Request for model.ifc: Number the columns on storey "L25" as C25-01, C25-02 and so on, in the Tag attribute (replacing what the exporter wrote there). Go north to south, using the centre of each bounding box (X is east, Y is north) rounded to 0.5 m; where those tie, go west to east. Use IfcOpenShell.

First a look at what the model holds.

```python
import ifcopenshell
import ifcopenshell.util.element
import ifcopenshell.util.placement

model = ifcopenshell.open("model.ifc")
print(model.schema)
storey = next(s for s in model.by_type("IfcBuildingStorey") if s.Name == "L25")
columns = [e for e in ifcopenshell.util.element.get_decomposition(storey) if e.is_a("IfcColumn")]
for e in sorted(columns, key=lambda e: e.id()):
    origin = ifcopenshell.util.placement.get_local_placement(e.ObjectPlacement)[:3, 3]
    print(e.id(), e.Tag, e.Name, origin.round(2) + 0.0, sep=" | ")
```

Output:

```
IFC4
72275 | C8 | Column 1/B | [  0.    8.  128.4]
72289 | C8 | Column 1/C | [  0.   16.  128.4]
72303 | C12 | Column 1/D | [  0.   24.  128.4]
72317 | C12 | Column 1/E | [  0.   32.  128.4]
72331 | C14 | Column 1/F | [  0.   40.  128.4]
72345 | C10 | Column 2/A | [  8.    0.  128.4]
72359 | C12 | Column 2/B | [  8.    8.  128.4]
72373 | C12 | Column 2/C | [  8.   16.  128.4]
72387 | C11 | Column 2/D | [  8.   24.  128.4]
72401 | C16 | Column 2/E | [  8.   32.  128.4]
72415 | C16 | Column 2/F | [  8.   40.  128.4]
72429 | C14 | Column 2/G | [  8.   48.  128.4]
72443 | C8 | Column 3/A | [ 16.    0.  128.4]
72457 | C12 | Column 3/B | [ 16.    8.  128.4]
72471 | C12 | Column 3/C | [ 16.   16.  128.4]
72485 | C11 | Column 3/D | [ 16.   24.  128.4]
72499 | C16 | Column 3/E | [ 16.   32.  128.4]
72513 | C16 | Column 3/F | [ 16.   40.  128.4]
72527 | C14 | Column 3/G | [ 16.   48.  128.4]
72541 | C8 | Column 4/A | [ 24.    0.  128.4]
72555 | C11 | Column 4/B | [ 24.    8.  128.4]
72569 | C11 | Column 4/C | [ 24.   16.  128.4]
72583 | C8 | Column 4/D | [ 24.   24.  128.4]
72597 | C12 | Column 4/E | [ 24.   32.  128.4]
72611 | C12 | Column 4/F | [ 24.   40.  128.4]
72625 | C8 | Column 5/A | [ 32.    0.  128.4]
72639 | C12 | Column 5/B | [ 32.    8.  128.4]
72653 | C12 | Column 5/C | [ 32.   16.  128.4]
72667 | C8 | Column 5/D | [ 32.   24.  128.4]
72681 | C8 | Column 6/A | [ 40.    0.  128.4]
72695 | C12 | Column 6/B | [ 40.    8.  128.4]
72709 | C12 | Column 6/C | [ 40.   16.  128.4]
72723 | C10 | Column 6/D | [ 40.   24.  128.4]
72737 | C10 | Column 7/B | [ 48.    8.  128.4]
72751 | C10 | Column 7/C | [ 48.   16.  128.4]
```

```python
import ifcopenshell
import ifcopenshell.geom
import ifcopenshell.util.element
import ifcopenshell.util.shape

model = ifcopenshell.open("model.ifc")
settings = ifcopenshell.geom.settings()
settings.set("use-world-coords", True)


def centre(element):
    shape = ifcopenshell.geom.create_shape(settings, element)
    return ifcopenshell.util.shape.get_bbox_centroid(shape.geometry)


storey = next(s for s in model.by_type("IfcBuildingStorey") if s.Name == "L25")
columns = [e for e in ifcopenshell.util.element.get_decomposition(storey) if e.is_a("IfcColumn")]

# Insertion points can sit at a corner or the storey origin, so sort by the geometry (in metres).
centres = {e: centre(e) for e in columns}
columns.sort(key=lambda e: (-round(centres[e][1] / 0.5), centres[e][0]))

for i, e in enumerate(columns, start=1):
    number = f"C25-{i:02d}"
    e.Tag = number
    print(e.id(), number)

model.write("model-out.ifc")
```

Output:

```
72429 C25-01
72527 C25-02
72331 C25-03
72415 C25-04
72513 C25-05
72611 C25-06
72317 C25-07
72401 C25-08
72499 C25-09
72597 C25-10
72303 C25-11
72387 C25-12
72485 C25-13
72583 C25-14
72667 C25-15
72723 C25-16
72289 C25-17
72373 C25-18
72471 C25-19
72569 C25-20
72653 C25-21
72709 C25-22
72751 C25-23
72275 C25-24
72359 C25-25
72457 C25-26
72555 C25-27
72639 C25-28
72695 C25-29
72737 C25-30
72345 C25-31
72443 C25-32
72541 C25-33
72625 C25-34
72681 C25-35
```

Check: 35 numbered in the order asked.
